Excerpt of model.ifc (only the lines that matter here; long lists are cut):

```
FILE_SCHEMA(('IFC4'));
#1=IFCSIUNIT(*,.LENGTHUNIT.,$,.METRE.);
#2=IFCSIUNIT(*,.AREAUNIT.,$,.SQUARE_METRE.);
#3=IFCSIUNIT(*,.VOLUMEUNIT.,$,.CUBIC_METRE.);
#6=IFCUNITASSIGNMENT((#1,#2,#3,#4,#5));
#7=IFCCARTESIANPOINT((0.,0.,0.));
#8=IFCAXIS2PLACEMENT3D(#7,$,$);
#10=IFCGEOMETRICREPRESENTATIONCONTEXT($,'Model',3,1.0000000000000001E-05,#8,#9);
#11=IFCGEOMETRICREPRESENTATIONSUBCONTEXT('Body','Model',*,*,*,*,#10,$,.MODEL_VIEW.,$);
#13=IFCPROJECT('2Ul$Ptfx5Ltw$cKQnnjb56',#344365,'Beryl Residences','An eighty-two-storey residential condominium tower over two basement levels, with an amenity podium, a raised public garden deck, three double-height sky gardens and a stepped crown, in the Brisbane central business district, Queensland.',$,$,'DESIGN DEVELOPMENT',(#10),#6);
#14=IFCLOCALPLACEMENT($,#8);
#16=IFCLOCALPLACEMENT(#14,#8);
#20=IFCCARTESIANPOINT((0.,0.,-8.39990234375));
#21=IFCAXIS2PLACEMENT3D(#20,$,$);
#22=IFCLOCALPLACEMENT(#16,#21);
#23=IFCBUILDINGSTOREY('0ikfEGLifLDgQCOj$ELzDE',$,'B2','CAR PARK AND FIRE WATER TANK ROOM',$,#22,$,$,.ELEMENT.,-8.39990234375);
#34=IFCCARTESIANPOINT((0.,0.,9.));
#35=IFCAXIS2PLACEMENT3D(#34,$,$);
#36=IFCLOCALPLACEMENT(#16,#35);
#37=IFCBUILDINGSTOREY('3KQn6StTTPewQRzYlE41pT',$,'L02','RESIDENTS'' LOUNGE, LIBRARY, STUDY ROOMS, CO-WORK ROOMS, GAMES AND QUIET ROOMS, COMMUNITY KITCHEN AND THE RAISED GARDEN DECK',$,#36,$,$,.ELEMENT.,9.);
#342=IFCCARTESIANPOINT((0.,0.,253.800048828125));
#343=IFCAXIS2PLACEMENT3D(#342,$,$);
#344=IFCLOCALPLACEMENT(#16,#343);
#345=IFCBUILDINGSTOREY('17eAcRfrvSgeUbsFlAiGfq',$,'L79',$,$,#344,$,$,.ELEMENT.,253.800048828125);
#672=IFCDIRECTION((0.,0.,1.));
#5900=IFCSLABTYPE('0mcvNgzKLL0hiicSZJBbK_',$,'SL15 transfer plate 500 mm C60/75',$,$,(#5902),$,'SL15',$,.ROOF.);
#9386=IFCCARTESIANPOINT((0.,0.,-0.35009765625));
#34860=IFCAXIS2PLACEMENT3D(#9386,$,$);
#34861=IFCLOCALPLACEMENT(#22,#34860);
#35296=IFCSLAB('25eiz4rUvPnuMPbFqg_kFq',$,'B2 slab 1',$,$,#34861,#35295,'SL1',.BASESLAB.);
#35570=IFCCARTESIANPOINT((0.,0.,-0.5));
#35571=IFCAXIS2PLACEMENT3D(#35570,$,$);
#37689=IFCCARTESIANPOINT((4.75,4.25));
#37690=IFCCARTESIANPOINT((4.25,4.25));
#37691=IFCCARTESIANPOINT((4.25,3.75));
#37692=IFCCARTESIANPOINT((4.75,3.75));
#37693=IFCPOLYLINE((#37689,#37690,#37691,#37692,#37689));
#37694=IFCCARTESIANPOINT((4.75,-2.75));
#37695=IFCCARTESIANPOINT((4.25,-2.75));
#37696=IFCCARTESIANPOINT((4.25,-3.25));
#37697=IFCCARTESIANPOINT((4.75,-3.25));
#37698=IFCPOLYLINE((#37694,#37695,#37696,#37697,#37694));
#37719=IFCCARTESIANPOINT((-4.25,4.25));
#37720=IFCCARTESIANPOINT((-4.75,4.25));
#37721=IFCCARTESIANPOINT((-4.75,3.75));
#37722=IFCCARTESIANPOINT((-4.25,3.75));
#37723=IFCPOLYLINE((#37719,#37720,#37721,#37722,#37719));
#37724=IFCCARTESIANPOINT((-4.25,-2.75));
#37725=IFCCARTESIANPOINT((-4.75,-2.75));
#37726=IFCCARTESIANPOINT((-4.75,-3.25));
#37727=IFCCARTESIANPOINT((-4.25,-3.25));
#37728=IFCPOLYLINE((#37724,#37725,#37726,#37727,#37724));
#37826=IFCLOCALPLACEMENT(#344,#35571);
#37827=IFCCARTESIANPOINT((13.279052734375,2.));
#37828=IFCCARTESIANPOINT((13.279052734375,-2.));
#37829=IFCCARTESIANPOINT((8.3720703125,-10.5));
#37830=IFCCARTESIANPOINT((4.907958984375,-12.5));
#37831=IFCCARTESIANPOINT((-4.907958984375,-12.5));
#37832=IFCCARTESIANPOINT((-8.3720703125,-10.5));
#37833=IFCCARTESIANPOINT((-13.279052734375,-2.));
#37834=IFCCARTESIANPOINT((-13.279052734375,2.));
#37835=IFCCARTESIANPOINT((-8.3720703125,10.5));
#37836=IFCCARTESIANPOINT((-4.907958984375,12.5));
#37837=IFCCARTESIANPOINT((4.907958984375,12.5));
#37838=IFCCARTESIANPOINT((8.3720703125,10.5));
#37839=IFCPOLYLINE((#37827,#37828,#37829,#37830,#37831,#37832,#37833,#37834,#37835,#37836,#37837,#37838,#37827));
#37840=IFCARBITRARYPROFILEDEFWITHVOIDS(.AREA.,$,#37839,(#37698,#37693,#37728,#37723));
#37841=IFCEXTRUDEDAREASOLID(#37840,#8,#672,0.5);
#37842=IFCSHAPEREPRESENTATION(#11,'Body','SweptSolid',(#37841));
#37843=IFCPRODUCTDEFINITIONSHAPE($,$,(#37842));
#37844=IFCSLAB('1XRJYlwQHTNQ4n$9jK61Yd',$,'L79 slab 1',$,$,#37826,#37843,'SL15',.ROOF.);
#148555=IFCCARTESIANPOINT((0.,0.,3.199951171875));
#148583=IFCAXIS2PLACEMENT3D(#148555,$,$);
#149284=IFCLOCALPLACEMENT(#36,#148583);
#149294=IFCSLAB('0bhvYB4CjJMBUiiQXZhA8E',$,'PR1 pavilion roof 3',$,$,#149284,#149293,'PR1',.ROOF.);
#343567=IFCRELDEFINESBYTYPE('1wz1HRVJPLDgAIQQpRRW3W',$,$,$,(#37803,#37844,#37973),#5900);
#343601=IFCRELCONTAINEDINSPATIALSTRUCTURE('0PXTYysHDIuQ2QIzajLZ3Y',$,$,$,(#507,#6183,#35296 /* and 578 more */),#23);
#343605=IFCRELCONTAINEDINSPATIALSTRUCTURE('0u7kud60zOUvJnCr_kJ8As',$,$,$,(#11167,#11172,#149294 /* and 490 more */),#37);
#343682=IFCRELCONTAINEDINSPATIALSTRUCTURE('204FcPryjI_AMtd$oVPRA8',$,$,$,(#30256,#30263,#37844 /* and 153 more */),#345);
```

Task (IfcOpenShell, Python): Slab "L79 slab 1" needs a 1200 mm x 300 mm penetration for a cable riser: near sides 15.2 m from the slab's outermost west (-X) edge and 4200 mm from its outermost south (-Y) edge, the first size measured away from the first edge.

```python
import numpy as np
import ifcopenshell
import ifcopenshell.api.feature
import ifcopenshell.api.geometry
import ifcopenshell.api.root
import ifcopenshell.geom
import ifcopenshell.util.placement
import ifcopenshell.util.representation
import ifcopenshell.util.shape
import ifcopenshell.util.unit

model = ifcopenshell.open("model.ifc")
unit_scale = ifcopenshell.util.unit.calculate_unit_scale(model)
settings = ifcopenshell.geom.settings()


def volume(element):
    """Net volume in cubic metres, openings subtracted."""
    shape = ifcopenshell.geom.create_shape(settings, element)
    return ifcopenshell.util.shape.get_volume(shape.geometry)


slab = model.by_id(37844)
before = volume(slab)

# Extent in the slab's own axes, in metres. The edges named are its -X and -Y sides.
slab_shape = ifcopenshell.geom.create_shape(settings, slab)
vertices = ifcopenshell.util.shape.get_vertices(slab_shape.geometry)
x_min, y_min, bottom = vertices.min(axis=0)
top = vertices[:, 2].max()

opening = ifcopenshell.api.root.create_entity(model, ifc_class="IfcOpeningElement", name="Cable riser opening", predefined_type="OPENING")
context = ifcopenshell.util.representation.get_context(model, "Model", "Body", "MODEL_VIEW")
width, depth = 1.2, 0.3
outline = [(0.0, 0.0), (width, 0.0), (width, depth), (0.0, depth), (0.0, 0.0)]
# Overshoot both faces by 50 mm so the cut is clean.
shape = ifcopenshell.api.geometry.add_slab_representation(
    model, context=context, depth=top - bottom + 0.1, polyline=outline
)
ifcopenshell.api.geometry.assign_representation(model, product=opening, representation=shape)

matrix = ifcopenshell.util.placement.get_local_placement(slab.ObjectPlacement)
matrix[:, 3] = matrix @ np.append(np.array([x_min + 15.2, y_min + 4.2, bottom - 0.05]) / unit_scale, 1.0)
ifcopenshell.api.geometry.edit_object_placement(model, product=opening, matrix=matrix, is_si=False)
ifcopenshell.api.feature.add_feature(model, feature=opening, element=slab)

after = volume(slab)

print(f"slab volume {before:.3f} -> {after:.3f} m3")

model.write("model_updated.ifc")
```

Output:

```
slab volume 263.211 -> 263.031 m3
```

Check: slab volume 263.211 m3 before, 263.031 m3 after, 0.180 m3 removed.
